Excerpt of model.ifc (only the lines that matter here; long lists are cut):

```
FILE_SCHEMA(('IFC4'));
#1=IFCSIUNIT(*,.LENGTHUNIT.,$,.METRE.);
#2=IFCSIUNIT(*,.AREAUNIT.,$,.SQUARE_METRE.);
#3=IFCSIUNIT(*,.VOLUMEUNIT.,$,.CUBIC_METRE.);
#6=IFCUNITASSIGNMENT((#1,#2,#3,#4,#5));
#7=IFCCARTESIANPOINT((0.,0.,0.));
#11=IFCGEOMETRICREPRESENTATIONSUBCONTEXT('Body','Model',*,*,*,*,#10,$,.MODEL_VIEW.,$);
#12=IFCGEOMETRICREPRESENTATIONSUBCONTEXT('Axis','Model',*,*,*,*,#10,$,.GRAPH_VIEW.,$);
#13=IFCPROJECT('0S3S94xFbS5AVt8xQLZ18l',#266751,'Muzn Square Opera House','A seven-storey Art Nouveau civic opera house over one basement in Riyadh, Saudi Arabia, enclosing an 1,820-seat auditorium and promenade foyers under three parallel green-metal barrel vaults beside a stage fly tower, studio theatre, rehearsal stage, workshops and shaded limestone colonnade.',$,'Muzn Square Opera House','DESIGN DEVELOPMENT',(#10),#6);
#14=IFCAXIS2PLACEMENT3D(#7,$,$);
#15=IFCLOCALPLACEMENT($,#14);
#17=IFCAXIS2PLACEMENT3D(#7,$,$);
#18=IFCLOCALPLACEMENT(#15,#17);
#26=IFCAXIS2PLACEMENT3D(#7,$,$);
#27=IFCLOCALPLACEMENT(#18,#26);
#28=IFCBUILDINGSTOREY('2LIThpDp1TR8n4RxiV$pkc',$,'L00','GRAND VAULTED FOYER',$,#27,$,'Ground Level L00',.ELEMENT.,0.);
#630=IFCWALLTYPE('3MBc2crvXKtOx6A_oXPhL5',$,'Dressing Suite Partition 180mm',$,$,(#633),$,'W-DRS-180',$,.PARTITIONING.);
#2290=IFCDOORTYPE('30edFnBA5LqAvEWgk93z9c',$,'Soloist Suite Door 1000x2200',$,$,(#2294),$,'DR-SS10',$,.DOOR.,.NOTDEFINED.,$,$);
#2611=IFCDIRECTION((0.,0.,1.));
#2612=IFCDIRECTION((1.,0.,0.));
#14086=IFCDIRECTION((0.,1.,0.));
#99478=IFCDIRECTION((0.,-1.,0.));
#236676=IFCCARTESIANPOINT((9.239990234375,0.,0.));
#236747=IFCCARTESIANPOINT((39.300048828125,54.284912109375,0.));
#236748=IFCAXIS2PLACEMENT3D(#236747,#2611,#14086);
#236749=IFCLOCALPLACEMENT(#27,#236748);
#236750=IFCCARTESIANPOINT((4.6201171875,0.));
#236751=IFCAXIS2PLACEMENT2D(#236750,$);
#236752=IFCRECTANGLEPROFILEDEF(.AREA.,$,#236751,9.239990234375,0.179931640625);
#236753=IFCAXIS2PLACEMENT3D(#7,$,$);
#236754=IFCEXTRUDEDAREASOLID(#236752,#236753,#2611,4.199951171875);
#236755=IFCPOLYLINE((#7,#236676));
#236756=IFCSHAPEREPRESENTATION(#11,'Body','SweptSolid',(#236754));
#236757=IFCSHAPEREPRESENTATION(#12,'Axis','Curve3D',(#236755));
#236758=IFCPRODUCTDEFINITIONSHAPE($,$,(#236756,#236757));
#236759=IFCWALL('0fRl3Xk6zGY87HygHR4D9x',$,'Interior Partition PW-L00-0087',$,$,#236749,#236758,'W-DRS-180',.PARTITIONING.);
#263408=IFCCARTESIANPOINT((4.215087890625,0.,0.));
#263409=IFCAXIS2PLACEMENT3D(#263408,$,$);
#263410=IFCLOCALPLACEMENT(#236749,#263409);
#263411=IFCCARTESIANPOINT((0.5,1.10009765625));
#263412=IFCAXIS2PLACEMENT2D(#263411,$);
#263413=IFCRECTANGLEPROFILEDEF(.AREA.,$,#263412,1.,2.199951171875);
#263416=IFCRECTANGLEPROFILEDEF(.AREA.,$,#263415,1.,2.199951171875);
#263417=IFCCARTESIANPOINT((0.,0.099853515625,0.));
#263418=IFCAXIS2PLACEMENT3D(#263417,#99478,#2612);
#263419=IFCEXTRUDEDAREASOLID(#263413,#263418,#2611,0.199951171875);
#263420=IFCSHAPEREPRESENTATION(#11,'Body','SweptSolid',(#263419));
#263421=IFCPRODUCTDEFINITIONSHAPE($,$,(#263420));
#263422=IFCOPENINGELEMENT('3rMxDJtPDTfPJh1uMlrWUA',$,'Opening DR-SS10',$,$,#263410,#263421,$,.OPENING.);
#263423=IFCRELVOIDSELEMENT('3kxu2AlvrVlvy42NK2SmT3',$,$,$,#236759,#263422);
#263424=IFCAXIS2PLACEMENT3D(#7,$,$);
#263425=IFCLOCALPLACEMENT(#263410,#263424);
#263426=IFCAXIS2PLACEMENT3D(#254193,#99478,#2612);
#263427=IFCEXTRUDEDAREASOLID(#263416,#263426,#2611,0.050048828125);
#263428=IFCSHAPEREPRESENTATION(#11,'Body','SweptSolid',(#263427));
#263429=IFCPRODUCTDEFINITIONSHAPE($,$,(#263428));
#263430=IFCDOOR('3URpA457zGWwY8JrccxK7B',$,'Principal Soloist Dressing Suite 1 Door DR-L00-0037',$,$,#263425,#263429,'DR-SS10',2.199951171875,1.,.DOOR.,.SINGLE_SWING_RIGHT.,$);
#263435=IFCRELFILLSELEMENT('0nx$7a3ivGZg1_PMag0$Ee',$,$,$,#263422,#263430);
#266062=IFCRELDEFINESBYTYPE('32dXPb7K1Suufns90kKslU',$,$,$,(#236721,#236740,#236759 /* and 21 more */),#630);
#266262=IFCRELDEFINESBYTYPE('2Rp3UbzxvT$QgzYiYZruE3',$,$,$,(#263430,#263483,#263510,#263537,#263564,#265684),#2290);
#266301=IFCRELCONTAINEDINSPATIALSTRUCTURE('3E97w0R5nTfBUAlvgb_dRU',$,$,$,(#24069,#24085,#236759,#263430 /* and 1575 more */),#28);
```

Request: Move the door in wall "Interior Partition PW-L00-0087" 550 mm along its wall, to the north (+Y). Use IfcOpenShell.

```python
import ifcopenshell
import ifcopenshell.api.geometry
import ifcopenshell.util.placement
import ifcopenshell.util.unit

model = ifcopenshell.open("model.ifc")
unit_scale = ifcopenshell.util.unit.calculate_unit_scale(model)

door = model.by_guid("3URpA457zGWwY8JrccxK7B")
opening = door.FillsVoids[0].RelatingOpeningElement
wall = opening.VoidsElements[0].RelatingBuildingElement

wall_matrix = ifcopenshell.util.placement.get_local_placement(wall.ObjectPlacement)
shift = wall_matrix[:3, 0] * 0.55 / unit_scale
before = ifcopenshell.util.placement.get_local_placement(door.ObjectPlacement)[:3, 3].copy()

# The door is placed relative to its opening, so it follows when the opening moves.
matrix = ifcopenshell.util.placement.get_local_placement(opening.ObjectPlacement)
matrix[:3, 3] += shift
ifcopenshell.api.geometry.edit_object_placement(
    model, product=opening, matrix=matrix, is_si=False, should_transform_children=True
)

after = ifcopenshell.util.placement.get_local_placement(door.ObjectPlacement)[:3, 3]
print("door moved by", (after - before).round(3) + 0.0)

model.write("model_rev.ifc")
```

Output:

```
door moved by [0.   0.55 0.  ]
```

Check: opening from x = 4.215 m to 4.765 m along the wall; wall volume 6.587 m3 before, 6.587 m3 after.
